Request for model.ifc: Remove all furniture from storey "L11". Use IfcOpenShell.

First a look at what the model holds.

```python
import ifcopenshell
import ifcopenshell.util.element

model = ifcopenshell.open("model.ifc")
print(model.schema)
storey = next(s for s in model.by_type("IfcBuildingStorey") if s.Name == "L11")
furniture = [e for e in ifcopenshell.util.element.get_decomposition(storey) if e.is_a("IfcFurnishingElement")]
seen = {}
for e in furniture:
    element_type = ifcopenshell.util.element.get_type(e)
    name = element_type.Name if element_type not in (None, e) else None
    seen[name] = seen.get(name, 0) + 1
for name, count in sorted(seen.items(), key=str):
    print(count, "x", name)
```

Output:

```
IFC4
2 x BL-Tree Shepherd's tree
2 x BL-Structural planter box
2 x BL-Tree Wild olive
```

```python
import ifcopenshell
import ifcopenshell.api.root
import ifcopenshell.util.element

model = ifcopenshell.open("model.ifc")

storey = next(s for s in model.by_type("IfcBuildingStorey") if s.Name == "L11")
furniture = [e for e in ifcopenshell.util.element.get_decomposition(storey) if e.is_a("IfcFurnishingElement")]

for e in furniture:
    ifcopenshell.api.root.remove_product(model, product=e)
print(len(furniture), "removed")

model.write("model_rev.ifc")
```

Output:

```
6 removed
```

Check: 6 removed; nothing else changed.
